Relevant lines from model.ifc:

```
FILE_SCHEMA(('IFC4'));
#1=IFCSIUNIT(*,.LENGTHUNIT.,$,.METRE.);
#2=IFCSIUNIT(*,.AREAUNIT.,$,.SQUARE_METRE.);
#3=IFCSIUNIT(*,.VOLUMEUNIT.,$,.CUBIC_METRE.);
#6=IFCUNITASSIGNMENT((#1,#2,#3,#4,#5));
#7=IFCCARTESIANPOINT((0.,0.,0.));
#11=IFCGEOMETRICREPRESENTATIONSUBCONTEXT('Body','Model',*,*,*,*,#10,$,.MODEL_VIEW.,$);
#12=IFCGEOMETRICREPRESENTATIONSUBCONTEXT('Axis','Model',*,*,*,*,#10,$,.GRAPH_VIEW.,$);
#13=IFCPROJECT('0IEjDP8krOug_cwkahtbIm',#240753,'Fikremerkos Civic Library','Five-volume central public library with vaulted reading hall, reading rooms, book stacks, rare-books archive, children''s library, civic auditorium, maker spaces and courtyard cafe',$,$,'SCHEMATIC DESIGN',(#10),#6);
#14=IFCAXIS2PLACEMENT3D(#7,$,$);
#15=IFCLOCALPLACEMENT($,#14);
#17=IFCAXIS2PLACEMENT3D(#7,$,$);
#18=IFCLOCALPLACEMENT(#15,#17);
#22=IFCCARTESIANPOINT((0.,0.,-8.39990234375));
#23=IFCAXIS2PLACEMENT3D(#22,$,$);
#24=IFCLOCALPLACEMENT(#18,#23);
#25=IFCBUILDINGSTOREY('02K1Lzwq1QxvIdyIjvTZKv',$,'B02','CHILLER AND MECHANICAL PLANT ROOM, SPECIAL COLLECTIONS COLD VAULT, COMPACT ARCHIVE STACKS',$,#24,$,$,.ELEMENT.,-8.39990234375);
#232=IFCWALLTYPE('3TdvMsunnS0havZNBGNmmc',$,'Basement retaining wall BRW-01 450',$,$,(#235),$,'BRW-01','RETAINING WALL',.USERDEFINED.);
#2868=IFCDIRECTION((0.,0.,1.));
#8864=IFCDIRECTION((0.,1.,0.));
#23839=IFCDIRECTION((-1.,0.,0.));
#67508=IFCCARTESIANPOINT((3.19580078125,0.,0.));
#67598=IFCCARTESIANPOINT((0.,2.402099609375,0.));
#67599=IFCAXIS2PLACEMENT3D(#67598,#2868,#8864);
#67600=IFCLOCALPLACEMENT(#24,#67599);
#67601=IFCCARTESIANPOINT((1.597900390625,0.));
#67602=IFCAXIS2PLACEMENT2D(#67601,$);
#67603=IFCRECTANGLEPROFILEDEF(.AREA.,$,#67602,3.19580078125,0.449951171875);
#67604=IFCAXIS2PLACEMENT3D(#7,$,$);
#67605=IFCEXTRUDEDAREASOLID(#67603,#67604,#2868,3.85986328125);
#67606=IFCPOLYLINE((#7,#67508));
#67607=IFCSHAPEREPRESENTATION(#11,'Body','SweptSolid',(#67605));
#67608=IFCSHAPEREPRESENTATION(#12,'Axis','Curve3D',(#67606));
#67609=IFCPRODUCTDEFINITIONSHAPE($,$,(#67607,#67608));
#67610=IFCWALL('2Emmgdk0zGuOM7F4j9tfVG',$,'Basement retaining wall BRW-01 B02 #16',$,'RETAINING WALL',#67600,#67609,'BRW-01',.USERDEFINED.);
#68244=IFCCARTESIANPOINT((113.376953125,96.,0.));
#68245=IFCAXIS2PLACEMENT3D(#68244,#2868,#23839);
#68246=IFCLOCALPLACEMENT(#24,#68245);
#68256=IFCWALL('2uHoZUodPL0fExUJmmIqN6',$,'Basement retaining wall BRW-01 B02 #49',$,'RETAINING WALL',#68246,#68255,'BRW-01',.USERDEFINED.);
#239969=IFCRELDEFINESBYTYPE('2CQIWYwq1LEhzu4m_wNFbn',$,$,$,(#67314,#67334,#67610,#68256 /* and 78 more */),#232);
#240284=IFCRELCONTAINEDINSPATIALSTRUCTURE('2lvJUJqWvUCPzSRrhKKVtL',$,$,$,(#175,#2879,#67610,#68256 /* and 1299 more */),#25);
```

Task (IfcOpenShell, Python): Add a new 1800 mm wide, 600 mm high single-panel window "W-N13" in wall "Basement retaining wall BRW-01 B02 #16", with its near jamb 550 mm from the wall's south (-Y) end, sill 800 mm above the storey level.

```python
import numpy as np
import ifcopenshell
import ifcopenshell.api.feature
import ifcopenshell.api.geometry
import ifcopenshell.api.root
import ifcopenshell.api.spatial
import ifcopenshell.geom
import ifcopenshell.util.element
import ifcopenshell.util.placement
import ifcopenshell.util.representation
import ifcopenshell.util.shape
import ifcopenshell.util.unit

model = ifcopenshell.open("model.ifc")
unit_scale = ifcopenshell.util.unit.calculate_unit_scale(model)
settings = ifcopenshell.geom.settings()


def volume(element):
    """Net volume in cubic metres, openings subtracted."""
    shape = ifcopenshell.geom.create_shape(settings, element)
    return ifcopenshell.util.shape.get_volume(shape.geometry)


wall = model.by_guid("2Emmgdk0zGuOM7F4j9tfVG")
storey = ifcopenshell.util.element.get_container(wall, ifc_class="IfcBuildingStorey")
context = ifcopenshell.util.representation.get_context(model, "Model", "Body", "MODEL_VIEW")
before = volume(wall)

width, height, from_end, sill = 1.8, 0.6, 0.55, 0.8  # metres

# The wall runs along its own X axis, and the end named is its -X end.
wall_shape = ifcopenshell.geom.create_shape(settings, wall)
x, y, z = ifcopenshell.util.shape.get_vertices(wall_shape.geometry).T
start = x.min() + from_end
face, thickness = float(y.min()), float(y.max() - y.min())
wall_matrix = ifcopenshell.util.placement.get_local_placement(wall.ObjectPlacement)
level = ifcopenshell.util.placement.get_local_placement(storey.ObjectPlacement)[2, 3]


def in_wall(x, y):
    """Placement at x, y metres in the wall's axes, at sill height."""
    matrix = wall_matrix.copy()
    matrix[:, 3] = wall_matrix @ np.array([x / unit_scale, y / unit_scale, 0.0, 1.0])
    matrix[2, 3] = level + sill / unit_scale
    return matrix


# Opening: a box that overshoots both wall faces by 50 mm.
opening = ifcopenshell.api.root.create_entity(model, ifc_class="IfcOpeningElement", predefined_type="OPENING")
box = ifcopenshell.api.geometry.add_wall_representation(
    model, context=context, length=width, height=height, thickness=thickness + 0.1
)
ifcopenshell.api.geometry.assign_representation(model, product=opening, representation=box)
ifcopenshell.api.geometry.edit_object_placement(model, product=opening, matrix=in_wall(start, face - 0.05), is_si=False)
ifcopenshell.api.feature.add_feature(model, feature=opening, element=wall)

window = ifcopenshell.api.root.create_entity(model, ifc_class="IfcWindow", name="W-N13", predefined_type="WINDOW")
window.OverallWidth, window.OverallHeight = width / unit_scale, height / unit_scale
window.PartitioningType = "SINGLE_PANEL"
body = ifcopenshell.api.geometry.add_window_representation(
    model,
    context=context,
    overall_width=window.OverallWidth,
    overall_height=window.OverallHeight,
    partition_type="SINGLE_PANEL",
)
ifcopenshell.api.geometry.assign_representation(model, product=window, representation=body)
ifcopenshell.api.spatial.assign_container(model, products=[window], relating_structure=storey)
ifcopenshell.api.feature.add_filling(model, opening=opening, element=window)

# Centre the window in the wall's thickness.
ifcopenshell.api.geometry.edit_object_placement(model, product=window, matrix=in_wall(start, face), is_si=False)
window_shape = ifcopenshell.geom.create_shape(settings, window)
depth = ifcopenshell.util.shape.get_vertices(window_shape.geometry)[:, 1]
offset = face + thickness / 2 - (depth.min() + depth.max()) / 2
ifcopenshell.api.geometry.edit_object_placement(model, product=window, matrix=in_wall(start, offset), is_si=False)

after = volume(wall)

print(f"wall volume {before:.3f} -> {after:.3f} m3")

model.write("model-out.ifc")
```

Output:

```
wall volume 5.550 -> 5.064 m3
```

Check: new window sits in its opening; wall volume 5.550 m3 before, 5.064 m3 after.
